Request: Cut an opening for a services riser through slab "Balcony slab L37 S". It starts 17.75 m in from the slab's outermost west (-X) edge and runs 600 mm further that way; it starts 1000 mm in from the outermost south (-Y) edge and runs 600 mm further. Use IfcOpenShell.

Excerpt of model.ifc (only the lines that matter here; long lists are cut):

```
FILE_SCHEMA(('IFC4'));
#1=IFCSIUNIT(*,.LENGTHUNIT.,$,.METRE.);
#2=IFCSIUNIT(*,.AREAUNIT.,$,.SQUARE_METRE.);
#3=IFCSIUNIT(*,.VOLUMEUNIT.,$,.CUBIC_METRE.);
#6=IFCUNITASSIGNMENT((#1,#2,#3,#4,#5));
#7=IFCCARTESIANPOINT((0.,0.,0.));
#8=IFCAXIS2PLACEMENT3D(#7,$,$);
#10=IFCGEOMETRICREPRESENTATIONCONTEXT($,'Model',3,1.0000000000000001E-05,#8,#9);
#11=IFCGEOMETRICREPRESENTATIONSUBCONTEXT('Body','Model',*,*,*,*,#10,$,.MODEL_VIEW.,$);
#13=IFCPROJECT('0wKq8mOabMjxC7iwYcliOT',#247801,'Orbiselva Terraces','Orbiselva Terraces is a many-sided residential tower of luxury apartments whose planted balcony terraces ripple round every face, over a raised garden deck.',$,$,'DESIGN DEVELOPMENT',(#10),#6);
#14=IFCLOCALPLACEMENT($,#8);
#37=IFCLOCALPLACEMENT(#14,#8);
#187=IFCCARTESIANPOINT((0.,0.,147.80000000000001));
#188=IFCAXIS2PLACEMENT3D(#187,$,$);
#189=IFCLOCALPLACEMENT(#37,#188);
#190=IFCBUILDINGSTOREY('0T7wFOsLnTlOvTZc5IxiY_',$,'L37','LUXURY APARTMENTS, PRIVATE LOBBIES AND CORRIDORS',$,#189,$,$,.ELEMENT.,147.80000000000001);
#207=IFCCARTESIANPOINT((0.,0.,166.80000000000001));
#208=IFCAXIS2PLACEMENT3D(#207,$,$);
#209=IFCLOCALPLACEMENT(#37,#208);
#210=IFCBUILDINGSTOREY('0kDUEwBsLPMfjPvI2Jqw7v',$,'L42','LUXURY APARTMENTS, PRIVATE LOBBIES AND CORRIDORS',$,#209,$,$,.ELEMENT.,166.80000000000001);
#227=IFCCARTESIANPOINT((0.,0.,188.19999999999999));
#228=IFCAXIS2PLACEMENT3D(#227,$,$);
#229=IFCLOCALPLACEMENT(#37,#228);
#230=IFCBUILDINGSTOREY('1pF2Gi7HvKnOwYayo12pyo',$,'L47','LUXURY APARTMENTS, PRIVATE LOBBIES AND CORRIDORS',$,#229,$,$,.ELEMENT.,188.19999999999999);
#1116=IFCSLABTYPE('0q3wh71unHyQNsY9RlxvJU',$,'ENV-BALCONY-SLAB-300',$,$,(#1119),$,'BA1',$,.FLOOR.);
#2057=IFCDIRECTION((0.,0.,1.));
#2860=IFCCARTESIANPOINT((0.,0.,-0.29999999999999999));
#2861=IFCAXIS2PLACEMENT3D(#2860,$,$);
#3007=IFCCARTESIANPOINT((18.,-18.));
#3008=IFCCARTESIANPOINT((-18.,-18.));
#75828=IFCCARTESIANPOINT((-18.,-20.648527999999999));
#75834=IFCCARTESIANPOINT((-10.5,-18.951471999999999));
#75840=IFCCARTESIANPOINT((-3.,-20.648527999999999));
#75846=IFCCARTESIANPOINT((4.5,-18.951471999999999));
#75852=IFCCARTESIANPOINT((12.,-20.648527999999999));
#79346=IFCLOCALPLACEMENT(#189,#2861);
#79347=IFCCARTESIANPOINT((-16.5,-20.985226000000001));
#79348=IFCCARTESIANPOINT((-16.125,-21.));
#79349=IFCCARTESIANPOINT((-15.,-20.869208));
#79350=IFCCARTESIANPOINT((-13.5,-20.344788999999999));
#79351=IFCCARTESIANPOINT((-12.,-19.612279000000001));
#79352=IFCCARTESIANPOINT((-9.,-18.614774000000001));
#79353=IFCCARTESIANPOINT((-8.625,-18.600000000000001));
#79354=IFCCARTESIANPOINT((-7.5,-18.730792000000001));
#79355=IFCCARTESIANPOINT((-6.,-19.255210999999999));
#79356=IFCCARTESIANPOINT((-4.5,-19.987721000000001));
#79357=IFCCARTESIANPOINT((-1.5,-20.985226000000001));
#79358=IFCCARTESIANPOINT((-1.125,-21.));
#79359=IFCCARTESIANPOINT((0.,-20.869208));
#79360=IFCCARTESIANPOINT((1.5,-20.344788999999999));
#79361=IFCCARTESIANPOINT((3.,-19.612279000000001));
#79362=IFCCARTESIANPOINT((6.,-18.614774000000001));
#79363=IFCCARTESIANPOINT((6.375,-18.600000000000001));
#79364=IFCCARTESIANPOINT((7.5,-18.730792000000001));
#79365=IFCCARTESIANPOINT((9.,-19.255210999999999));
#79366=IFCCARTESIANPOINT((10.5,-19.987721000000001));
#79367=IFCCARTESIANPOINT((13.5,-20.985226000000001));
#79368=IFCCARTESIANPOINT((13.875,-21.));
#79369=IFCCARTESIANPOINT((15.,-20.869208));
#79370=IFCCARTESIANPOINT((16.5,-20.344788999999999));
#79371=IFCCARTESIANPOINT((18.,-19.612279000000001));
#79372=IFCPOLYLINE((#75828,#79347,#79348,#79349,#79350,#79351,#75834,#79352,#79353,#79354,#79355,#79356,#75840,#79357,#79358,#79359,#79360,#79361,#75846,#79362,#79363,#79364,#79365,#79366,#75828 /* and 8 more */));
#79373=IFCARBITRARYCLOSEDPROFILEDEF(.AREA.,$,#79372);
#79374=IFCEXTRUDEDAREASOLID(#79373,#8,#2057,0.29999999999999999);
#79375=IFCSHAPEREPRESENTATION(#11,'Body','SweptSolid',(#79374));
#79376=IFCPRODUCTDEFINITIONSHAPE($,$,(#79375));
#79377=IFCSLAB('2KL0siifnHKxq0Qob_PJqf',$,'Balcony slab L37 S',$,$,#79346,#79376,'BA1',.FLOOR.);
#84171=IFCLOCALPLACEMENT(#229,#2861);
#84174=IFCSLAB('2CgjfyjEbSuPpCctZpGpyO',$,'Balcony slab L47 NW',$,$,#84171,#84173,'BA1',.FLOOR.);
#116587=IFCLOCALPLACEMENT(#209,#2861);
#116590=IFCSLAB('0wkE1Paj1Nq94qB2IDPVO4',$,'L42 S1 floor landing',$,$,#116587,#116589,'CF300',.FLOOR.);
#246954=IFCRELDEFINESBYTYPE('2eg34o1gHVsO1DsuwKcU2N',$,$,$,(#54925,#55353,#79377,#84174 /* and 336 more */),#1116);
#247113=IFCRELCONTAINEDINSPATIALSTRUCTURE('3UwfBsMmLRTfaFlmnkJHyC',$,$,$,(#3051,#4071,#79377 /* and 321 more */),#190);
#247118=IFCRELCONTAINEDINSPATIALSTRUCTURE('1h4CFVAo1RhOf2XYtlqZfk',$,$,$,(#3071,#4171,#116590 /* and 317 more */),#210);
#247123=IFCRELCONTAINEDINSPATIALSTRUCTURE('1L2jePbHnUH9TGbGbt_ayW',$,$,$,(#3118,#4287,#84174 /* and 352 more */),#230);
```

```python
import numpy as np
import ifcopenshell
import ifcopenshell.api.feature
import ifcopenshell.api.geometry
import ifcopenshell.api.root
import ifcopenshell.geom
import ifcopenshell.util.placement
import ifcopenshell.util.representation
import ifcopenshell.util.shape
import ifcopenshell.util.unit

model = ifcopenshell.open("model.ifc")
unit_scale = ifcopenshell.util.unit.calculate_unit_scale(model)
settings = ifcopenshell.geom.settings()


def volume(element):
    """Net volume in cubic metres, openings subtracted."""
    shape = ifcopenshell.geom.create_shape(settings, element)
    return ifcopenshell.util.shape.get_volume(shape.geometry)


slab = model.by_guid("2KL0siifnHKxq0Qob_PJqf")
before = volume(slab)

# Extent in the slab's own axes, in metres. The edges named are its -X and -Y sides.
slab_shape = ifcopenshell.geom.create_shape(settings, slab)
vertices = ifcopenshell.util.shape.get_vertices(slab_shape.geometry)
x_min, y_min, bottom = vertices.min(axis=0)
top = vertices[:, 2].max()

opening = ifcopenshell.api.root.create_entity(model, ifc_class="IfcOpeningElement", name="Services riser opening", predefined_type="OPENING")
context = ifcopenshell.util.representation.get_context(model, "Model", "Body", "MODEL_VIEW")
width, depth = 0.6, 0.6
outline = [(0.0, 0.0), (width, 0.0), (width, depth), (0.0, depth), (0.0, 0.0)]
# Overshoot both faces by 50 mm so the cut is clean.
shape = ifcopenshell.api.geometry.add_slab_representation(
    model, context=context, depth=top - bottom + 0.1, polyline=outline
)
ifcopenshell.api.geometry.assign_representation(model, product=opening, representation=shape)

matrix = ifcopenshell.util.placement.get_local_placement(slab.ObjectPlacement)
matrix[:, 3] = matrix @ np.append(np.array([x_min + 17.75, y_min + 1, bottom - 0.05]) / unit_scale, 1.0)
ifcopenshell.api.geometry.edit_object_placement(model, product=opening, matrix=matrix, is_si=False)
ifcopenshell.api.feature.add_feature(model, feature=opening, element=slab)

after = volume(slab)

print(f"slab volume {before:.3f} -> {after:.3f} m3")

model.write("model_v2.ifc")
```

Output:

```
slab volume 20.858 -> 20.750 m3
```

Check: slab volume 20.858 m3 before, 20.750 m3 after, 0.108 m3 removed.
